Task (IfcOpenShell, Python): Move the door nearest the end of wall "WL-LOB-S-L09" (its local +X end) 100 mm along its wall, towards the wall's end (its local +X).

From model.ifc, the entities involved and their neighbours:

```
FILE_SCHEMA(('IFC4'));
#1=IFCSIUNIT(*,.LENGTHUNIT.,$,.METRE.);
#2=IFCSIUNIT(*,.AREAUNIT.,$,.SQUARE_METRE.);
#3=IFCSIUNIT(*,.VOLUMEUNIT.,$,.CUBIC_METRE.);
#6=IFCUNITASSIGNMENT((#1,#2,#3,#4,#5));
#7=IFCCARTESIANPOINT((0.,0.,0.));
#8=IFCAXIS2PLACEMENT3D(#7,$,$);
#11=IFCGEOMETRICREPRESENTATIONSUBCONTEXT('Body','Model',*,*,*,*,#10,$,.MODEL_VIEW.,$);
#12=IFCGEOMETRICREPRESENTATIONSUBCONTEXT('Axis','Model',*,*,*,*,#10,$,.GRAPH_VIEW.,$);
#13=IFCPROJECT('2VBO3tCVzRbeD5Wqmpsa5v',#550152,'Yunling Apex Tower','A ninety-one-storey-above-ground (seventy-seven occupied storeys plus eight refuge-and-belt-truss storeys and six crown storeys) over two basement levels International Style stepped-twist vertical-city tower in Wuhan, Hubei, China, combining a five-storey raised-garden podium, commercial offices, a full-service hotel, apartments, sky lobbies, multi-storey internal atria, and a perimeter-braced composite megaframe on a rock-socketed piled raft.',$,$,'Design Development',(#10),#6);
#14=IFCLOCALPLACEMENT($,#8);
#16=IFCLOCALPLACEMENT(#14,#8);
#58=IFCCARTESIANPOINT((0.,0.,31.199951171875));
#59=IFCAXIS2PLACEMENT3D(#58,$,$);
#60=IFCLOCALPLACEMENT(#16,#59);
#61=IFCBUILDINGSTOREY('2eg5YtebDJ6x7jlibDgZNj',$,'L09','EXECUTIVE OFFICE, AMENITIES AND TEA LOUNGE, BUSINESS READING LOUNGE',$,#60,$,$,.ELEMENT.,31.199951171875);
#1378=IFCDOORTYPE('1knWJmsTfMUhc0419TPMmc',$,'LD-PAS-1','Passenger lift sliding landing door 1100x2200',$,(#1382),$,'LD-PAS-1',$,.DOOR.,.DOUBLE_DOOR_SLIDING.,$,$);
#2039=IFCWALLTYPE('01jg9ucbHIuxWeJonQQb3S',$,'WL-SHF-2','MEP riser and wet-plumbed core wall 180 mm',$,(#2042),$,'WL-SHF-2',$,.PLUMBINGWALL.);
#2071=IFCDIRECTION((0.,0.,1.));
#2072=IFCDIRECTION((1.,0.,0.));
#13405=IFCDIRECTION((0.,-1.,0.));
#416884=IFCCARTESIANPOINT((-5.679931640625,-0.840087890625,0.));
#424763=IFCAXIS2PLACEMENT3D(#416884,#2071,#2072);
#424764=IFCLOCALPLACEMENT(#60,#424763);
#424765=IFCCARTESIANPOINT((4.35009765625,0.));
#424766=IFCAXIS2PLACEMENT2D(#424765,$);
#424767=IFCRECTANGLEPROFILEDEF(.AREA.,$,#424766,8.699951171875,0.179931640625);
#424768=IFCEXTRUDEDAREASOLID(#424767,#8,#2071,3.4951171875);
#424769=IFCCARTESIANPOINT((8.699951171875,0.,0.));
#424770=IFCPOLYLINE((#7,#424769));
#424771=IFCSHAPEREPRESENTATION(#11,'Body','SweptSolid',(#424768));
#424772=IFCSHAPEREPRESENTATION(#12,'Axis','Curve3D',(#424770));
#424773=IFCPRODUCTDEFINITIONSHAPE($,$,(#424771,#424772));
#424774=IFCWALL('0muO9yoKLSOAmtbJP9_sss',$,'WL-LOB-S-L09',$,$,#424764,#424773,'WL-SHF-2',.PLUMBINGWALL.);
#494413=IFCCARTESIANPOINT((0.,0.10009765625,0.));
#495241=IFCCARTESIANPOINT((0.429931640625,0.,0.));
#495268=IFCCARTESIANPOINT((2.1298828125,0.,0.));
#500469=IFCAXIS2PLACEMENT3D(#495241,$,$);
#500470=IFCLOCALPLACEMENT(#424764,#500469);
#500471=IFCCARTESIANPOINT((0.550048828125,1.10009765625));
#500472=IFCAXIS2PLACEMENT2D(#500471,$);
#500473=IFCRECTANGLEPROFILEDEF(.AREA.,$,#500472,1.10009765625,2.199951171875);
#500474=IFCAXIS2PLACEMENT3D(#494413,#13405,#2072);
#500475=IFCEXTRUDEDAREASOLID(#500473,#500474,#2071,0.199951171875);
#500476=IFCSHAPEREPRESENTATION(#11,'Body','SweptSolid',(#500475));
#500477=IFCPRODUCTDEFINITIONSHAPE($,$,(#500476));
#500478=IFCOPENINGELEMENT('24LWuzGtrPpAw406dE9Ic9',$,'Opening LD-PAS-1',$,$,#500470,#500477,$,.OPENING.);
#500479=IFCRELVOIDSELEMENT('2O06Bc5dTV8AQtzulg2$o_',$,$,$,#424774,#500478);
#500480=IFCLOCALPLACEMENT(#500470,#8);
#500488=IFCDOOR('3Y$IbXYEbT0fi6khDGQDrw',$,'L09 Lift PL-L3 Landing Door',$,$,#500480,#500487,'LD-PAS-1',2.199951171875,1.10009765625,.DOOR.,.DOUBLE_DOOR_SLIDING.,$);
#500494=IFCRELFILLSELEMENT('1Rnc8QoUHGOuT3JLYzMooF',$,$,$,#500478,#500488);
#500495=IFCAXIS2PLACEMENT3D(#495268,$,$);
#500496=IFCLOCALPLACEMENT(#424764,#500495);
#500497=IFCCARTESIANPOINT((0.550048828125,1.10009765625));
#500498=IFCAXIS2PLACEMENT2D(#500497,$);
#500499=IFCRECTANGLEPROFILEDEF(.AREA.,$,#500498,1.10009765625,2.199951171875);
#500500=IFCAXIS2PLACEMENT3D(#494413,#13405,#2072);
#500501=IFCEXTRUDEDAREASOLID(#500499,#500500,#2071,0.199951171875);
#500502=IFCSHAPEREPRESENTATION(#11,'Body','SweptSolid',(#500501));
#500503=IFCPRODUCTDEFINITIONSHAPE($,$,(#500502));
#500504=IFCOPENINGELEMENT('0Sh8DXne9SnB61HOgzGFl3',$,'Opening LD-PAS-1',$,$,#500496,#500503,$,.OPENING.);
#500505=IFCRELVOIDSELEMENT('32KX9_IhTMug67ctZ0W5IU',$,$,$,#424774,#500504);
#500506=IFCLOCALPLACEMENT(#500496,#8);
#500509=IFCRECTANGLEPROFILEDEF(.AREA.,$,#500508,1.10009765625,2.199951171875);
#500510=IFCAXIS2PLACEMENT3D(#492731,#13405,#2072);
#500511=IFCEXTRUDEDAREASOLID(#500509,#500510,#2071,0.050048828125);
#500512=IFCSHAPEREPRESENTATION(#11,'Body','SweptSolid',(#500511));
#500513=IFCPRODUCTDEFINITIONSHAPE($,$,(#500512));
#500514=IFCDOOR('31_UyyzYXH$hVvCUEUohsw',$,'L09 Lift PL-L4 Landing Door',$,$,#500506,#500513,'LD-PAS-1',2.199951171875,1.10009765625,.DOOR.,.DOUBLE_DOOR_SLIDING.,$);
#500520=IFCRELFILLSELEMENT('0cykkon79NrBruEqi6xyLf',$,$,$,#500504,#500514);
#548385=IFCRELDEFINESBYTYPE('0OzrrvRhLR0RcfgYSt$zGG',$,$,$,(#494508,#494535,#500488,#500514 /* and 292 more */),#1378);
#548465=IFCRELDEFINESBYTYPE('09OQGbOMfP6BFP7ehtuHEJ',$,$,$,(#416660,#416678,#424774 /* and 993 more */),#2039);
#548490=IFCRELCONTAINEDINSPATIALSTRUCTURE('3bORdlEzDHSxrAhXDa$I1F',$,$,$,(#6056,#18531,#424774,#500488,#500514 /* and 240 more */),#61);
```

```python
import ifcopenshell
import ifcopenshell.api.geometry
import ifcopenshell.util.placement
import ifcopenshell.util.unit

model = ifcopenshell.open("model.ifc")
unit_scale = ifcopenshell.util.unit.calculate_unit_scale(model)

door = model.by_guid("31_UyyzYXH$hVvCUEUohsw")
opening = door.FillsVoids[0].RelatingOpeningElement
wall = opening.VoidsElements[0].RelatingBuildingElement

wall_matrix = ifcopenshell.util.placement.get_local_placement(wall.ObjectPlacement)
shift = wall_matrix[:3, 0] * 0.1 / unit_scale
before = ifcopenshell.util.placement.get_local_placement(door.ObjectPlacement)[:3, 3].copy()

# The door is placed relative to its opening, so it follows when the opening moves.
matrix = ifcopenshell.util.placement.get_local_placement(opening.ObjectPlacement)
matrix[:3, 3] += shift
ifcopenshell.api.geometry.edit_object_placement(
    model, product=opening, matrix=matrix, is_si=False, should_transform_children=True
)

after = ifcopenshell.util.placement.get_local_placement(door.ObjectPlacement)[:3, 3]
print("door moved by", (after - before).round(3) + 0.0)

model.write("model_edited.ifc")
```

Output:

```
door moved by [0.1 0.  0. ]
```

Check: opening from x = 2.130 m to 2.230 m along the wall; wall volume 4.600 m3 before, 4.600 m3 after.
